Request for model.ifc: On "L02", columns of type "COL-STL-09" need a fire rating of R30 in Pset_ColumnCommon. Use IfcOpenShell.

First a look at what the model holds.

```python
import ifcopenshell
import ifcopenshell.util.element

model = ifcopenshell.open("model.ifc")
print(model.schema)
storey = next(s for s in model.by_type("IfcBuildingStorey") if s.Name == "L02")
columns = [e for e in ifcopenshell.util.element.get_decomposition(storey) if e.is_a("IfcColumn")]
seen = {}
for e in columns:
    element_type = ifcopenshell.util.element.get_type(e)
    key = (element_type.Name if element_type != e and element_type else None, ifcopenshell.util.element.get_pset(e, "Pset_ColumnCommon", "FireRating"))
    seen[key] = seen.get(key, 0) + 1
for (name, value), count in sorted(seen.items(), key=str):
    print(count, "x", name, "|", value)
```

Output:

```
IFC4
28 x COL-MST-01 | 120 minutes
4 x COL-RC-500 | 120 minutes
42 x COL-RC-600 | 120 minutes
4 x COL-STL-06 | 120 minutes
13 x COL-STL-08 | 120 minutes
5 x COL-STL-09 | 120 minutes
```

```python
import ifcopenshell
import ifcopenshell.api.pset
import ifcopenshell.util.element

model = ifcopenshell.open("model.ifc")

storey = next(s for s in model.by_type("IfcBuildingStorey") if s.Name == "L02")
columns = [e for e in ifcopenshell.util.element.get_decomposition(storey) if e.is_a("IfcColumn")]

count = 0
for e in columns:
    element_type = ifcopenshell.util.element.get_type(e)
    if element_type in (None, e) or element_type.Name != "COL-STL-09":
        continue
    # add_pset returns the element's existing set when there is one.
    pset = ifcopenshell.api.pset.add_pset(model, product=e, name="Pset_ColumnCommon")
    ifcopenshell.api.pset.edit_pset(model, pset=pset, properties={"FireRating": "R30"})
    count += 1

print(count, "columns updated")

model.write("model_edited.ifc")
```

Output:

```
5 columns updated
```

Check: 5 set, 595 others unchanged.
